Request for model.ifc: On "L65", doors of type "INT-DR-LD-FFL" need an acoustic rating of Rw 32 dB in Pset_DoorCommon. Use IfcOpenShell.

First a look at what the model holds.

```python
import ifcopenshell
import ifcopenshell.util.element

model = ifcopenshell.open("model.ifc")
print(model.schema)
storey = next(s for s in model.by_type("IfcBuildingStorey") if s.Name == "L65")
doors = [e for e in ifcopenshell.util.element.get_decomposition(storey) if e.is_a("IfcDoor")]
seen = {}
for e in doors:
    element_type = ifcopenshell.util.element.get_type(e)
    key = (element_type.Name if element_type != e and element_type else None, ifcopenshell.util.element.get_pset(e, "Pset_DoorCommon", "AcousticRating"))
    seen[key] = seen.get(key, 0) + 1
for (name, value), count in sorted(seen.items(), key=str):
    print(count, "x", name, "|", value)
```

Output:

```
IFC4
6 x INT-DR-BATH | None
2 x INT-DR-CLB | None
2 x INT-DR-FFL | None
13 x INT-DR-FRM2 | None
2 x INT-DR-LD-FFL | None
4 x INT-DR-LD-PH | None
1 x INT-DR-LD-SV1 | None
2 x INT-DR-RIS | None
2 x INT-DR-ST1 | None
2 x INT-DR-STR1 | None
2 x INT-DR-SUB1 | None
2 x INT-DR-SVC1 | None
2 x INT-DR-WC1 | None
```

```python
import ifcopenshell
import ifcopenshell.api.pset
import ifcopenshell.util.element

model = ifcopenshell.open("model.ifc")

storey = next(s for s in model.by_type("IfcBuildingStorey") if s.Name == "L65")
doors = [e for e in ifcopenshell.util.element.get_decomposition(storey) if e.is_a("IfcDoor")]

count = 0
for e in doors:
    element_type = ifcopenshell.util.element.get_type(e)
    if element_type in (None, e) or element_type.Name != "INT-DR-LD-FFL":
        continue
    # add_pset returns the element's existing set when there is one.
    pset = ifcopenshell.api.pset.add_pset(model, product=e, name="Pset_DoorCommon")
    ifcopenshell.api.pset.edit_pset(model, pset=pset, properties={"AcousticRating": "Rw 32 dB"})
    count += 1

print(count, "doors updated")

model.write("model_updated.ifc")
```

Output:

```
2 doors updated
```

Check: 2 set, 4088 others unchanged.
